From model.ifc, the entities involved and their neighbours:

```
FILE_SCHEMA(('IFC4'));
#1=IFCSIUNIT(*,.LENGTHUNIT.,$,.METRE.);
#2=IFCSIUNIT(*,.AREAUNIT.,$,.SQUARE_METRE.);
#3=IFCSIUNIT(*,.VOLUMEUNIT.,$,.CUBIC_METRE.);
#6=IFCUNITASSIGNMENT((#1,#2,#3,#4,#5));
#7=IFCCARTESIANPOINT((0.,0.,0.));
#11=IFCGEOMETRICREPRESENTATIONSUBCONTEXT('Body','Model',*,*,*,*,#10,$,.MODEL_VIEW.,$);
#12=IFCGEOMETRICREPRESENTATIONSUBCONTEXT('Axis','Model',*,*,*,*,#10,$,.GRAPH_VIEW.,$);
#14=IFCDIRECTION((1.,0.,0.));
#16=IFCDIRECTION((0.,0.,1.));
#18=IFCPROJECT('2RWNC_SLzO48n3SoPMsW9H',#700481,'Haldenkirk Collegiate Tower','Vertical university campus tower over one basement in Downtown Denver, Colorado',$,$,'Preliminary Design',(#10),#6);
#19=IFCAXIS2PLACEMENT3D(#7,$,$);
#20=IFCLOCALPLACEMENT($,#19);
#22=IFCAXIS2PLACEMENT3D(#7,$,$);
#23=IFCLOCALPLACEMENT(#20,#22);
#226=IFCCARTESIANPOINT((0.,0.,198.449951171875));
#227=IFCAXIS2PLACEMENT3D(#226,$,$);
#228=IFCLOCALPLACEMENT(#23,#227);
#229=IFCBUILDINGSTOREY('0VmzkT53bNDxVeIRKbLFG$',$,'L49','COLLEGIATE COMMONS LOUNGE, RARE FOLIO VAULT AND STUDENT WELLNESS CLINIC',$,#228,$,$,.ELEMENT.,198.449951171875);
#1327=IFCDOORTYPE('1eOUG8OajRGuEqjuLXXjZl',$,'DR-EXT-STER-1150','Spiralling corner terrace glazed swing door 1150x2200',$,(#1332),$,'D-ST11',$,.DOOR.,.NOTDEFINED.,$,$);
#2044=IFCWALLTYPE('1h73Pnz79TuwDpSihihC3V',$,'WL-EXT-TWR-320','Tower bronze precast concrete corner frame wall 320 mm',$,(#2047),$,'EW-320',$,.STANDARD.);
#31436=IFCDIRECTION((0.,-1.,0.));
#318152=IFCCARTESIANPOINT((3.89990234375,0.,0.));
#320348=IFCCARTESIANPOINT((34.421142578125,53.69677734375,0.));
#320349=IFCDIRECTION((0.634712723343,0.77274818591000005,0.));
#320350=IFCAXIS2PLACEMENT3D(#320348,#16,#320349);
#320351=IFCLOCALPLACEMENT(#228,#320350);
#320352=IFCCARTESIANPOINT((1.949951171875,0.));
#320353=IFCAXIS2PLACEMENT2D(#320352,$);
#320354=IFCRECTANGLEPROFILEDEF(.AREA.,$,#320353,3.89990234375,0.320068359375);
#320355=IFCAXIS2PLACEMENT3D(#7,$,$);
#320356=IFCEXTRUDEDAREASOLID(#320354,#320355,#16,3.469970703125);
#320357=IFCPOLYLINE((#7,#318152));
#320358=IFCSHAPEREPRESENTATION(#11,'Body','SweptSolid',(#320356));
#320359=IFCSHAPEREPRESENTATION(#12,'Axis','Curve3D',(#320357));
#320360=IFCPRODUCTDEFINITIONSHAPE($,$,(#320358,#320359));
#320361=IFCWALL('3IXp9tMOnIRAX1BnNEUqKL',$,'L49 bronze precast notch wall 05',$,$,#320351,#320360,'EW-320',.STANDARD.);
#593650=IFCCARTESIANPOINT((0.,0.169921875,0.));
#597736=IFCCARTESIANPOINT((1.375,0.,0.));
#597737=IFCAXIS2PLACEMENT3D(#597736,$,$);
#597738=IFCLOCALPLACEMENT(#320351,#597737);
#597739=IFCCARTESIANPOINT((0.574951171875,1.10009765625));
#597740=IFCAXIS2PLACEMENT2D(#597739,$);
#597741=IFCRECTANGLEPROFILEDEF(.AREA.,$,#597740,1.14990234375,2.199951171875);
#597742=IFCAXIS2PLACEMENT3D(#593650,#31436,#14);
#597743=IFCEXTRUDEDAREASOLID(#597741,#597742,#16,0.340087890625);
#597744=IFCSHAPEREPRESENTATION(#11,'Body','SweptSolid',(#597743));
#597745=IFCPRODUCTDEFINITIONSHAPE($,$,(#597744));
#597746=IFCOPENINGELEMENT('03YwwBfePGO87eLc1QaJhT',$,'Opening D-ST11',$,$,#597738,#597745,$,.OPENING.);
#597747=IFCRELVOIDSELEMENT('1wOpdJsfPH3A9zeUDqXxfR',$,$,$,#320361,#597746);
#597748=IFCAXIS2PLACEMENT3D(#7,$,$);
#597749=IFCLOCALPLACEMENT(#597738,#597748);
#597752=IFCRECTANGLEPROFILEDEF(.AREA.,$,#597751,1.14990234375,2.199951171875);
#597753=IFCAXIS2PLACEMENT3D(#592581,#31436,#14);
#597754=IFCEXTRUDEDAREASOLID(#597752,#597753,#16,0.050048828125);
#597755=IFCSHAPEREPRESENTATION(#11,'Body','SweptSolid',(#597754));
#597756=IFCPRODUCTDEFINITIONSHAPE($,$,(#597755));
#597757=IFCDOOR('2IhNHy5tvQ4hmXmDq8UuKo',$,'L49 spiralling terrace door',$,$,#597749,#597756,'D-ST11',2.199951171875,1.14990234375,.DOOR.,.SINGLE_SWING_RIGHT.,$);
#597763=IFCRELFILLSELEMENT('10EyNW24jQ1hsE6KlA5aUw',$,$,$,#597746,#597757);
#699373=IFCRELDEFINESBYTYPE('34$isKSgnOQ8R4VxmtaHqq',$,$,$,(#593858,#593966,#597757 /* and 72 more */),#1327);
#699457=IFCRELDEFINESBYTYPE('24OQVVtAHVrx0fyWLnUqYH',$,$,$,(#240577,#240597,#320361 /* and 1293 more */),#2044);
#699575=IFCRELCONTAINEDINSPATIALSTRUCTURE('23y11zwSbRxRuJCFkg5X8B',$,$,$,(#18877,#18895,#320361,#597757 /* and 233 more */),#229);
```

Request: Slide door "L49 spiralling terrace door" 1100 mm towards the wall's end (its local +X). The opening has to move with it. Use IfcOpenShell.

```python
import ifcopenshell
import ifcopenshell.api.geometry
import ifcopenshell.util.placement
import ifcopenshell.util.unit

model = ifcopenshell.open("model.ifc")
unit_scale = ifcopenshell.util.unit.calculate_unit_scale(model)

door = model.by_guid("2IhNHy5tvQ4hmXmDq8UuKo")
opening = door.FillsVoids[0].RelatingOpeningElement
wall = opening.VoidsElements[0].RelatingBuildingElement

wall_matrix = ifcopenshell.util.placement.get_local_placement(wall.ObjectPlacement)
shift = wall_matrix[:3, 0] * 1.1 / unit_scale
before = ifcopenshell.util.placement.get_local_placement(door.ObjectPlacement)[:3, 3].copy()

# The door is placed relative to its opening, so it follows when the opening moves.
matrix = ifcopenshell.util.placement.get_local_placement(opening.ObjectPlacement)
matrix[:3, 3] += shift
ifcopenshell.api.geometry.edit_object_placement(
    model, product=opening, matrix=matrix, is_si=False, should_transform_children=True
)

after = ifcopenshell.util.placement.get_local_placement(door.ObjectPlacement)[:3, 3]
print("door moved by", (after - before).round(3) + 0.0)

model.write("model_v2.ifc")
```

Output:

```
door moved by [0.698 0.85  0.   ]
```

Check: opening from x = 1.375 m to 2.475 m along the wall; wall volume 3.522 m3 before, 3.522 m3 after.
